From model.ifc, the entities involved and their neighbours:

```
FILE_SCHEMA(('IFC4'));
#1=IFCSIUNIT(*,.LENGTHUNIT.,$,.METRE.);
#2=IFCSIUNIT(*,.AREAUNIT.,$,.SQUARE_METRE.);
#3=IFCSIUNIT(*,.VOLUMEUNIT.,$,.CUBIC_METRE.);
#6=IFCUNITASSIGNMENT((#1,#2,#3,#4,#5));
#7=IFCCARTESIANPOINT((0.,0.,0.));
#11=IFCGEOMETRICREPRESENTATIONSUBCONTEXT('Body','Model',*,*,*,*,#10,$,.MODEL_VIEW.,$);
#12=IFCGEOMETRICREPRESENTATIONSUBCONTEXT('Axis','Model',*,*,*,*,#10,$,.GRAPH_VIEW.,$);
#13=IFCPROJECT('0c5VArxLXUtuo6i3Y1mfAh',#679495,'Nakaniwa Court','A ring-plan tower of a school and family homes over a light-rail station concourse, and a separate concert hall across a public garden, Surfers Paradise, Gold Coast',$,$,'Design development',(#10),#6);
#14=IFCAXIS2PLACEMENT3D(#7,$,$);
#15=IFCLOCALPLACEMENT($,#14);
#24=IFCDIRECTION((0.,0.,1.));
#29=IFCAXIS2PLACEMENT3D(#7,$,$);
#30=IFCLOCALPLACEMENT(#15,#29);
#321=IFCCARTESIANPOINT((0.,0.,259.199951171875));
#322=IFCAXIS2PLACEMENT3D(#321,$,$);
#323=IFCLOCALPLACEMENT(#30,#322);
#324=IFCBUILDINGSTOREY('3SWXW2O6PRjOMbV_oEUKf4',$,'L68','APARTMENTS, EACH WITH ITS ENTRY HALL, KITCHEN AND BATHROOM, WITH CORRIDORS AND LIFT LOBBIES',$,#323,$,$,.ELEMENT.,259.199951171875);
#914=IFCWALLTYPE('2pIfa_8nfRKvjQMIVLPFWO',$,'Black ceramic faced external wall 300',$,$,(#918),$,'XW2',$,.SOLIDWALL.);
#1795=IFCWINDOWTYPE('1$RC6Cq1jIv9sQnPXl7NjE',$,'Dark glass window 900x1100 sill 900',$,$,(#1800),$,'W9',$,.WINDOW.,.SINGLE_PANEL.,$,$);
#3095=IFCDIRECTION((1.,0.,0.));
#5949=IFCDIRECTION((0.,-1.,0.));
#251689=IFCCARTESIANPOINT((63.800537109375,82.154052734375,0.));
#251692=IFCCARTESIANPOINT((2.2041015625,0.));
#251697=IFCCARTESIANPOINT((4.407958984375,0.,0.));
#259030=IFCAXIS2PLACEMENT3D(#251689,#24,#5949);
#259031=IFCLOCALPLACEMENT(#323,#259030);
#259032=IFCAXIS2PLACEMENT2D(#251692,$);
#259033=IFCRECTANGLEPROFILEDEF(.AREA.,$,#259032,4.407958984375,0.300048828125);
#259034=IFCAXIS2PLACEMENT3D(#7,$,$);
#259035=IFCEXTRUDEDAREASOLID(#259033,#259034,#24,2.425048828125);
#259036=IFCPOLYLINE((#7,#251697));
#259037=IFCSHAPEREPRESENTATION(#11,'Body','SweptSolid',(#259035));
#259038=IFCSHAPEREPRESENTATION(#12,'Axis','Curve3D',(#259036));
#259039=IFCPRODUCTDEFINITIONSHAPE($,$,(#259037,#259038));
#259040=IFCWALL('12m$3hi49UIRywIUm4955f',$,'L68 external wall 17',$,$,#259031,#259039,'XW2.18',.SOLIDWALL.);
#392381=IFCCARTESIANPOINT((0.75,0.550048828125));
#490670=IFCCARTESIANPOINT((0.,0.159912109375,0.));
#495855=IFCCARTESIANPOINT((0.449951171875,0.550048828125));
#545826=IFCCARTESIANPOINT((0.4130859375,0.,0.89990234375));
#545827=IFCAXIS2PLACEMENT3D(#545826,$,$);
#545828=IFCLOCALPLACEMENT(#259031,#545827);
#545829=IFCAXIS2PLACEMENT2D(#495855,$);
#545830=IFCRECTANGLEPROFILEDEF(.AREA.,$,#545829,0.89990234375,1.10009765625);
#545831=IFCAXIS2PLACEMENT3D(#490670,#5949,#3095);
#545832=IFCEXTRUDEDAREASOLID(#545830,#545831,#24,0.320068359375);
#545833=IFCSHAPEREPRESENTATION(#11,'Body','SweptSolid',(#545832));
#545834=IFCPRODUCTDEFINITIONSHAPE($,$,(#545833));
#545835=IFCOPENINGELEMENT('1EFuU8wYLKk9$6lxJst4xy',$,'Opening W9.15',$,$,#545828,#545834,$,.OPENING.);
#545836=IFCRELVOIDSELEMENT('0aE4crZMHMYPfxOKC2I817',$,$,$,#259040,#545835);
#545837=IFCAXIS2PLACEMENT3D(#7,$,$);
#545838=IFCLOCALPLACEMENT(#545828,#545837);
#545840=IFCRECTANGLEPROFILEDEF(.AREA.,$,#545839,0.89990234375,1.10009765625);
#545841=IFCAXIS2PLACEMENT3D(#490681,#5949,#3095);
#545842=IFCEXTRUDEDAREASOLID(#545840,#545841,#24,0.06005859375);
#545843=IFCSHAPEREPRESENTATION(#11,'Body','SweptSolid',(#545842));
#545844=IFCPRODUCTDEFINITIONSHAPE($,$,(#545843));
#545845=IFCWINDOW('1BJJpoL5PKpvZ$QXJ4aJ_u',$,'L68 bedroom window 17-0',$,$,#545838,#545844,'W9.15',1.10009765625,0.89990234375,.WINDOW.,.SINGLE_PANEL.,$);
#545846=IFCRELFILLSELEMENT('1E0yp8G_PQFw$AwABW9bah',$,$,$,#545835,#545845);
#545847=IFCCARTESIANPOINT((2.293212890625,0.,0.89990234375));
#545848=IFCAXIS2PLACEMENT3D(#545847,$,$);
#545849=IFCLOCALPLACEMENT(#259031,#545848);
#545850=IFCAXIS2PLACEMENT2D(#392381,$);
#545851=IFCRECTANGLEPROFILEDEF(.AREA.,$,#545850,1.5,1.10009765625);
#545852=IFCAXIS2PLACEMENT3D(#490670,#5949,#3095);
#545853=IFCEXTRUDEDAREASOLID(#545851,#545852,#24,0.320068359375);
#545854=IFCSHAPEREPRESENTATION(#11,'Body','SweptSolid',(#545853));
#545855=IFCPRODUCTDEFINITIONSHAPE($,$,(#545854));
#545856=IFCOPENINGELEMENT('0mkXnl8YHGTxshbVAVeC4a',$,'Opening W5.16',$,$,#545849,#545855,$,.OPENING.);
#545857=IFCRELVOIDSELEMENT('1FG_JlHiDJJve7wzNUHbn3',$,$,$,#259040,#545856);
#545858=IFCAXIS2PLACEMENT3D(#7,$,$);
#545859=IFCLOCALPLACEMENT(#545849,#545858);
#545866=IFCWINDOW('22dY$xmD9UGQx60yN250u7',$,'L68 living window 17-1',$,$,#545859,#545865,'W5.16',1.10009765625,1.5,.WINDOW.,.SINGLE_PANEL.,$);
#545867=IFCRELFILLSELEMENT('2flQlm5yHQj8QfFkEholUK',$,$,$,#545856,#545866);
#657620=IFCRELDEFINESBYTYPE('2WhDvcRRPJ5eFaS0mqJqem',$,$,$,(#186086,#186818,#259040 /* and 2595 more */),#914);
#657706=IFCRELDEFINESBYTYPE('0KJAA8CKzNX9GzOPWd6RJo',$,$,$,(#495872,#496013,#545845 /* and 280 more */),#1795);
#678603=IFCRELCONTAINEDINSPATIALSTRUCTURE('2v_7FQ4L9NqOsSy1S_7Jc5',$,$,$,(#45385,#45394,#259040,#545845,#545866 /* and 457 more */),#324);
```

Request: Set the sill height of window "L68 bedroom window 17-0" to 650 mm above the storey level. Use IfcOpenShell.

```python
import numpy as np
import ifcopenshell
import ifcopenshell.api.geometry
import ifcopenshell.geom
import ifcopenshell.util.element
import ifcopenshell.util.placement
import ifcopenshell.util.shape
import ifcopenshell.util.unit

model = ifcopenshell.open("model.ifc")
unit_scale = ifcopenshell.util.unit.calculate_unit_scale(model)

window = model.by_id(545845)
opening = window.FillsVoids[0].RelatingOpeningElement
storey = ifcopenshell.util.element.get_container(window, ifc_class="IfcBuildingStorey")
level = ifcopenshell.util.placement.get_local_placement(storey.ObjectPlacement)[2, 3]

# The opening's origin need not be at the sill, so measure its lowest point.
shape = ifcopenshell.geom.create_shape(ifcopenshell.geom.settings(), opening)
bottom = ifcopenshell.util.shape.get_shape_bottom_elevation(shape, shape.geometry) / unit_scale
dz = level + 0.65 / unit_scale - bottom

shift = np.array([0.0, 0.0, dz])
# The window is placed relative to its opening, so it follows when the opening moves.
matrix = ifcopenshell.util.placement.get_local_placement(opening.ObjectPlacement)
matrix[:3, 3] += shift
ifcopenshell.api.geometry.edit_object_placement(
    model, product=opening, matrix=matrix, is_si=False, should_transform_children=True
)

print(f"moved by {dz * unit_scale:+.3f} m")

model.write("model_rev.ifc")
```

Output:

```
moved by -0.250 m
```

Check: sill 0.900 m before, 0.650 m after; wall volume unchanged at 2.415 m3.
